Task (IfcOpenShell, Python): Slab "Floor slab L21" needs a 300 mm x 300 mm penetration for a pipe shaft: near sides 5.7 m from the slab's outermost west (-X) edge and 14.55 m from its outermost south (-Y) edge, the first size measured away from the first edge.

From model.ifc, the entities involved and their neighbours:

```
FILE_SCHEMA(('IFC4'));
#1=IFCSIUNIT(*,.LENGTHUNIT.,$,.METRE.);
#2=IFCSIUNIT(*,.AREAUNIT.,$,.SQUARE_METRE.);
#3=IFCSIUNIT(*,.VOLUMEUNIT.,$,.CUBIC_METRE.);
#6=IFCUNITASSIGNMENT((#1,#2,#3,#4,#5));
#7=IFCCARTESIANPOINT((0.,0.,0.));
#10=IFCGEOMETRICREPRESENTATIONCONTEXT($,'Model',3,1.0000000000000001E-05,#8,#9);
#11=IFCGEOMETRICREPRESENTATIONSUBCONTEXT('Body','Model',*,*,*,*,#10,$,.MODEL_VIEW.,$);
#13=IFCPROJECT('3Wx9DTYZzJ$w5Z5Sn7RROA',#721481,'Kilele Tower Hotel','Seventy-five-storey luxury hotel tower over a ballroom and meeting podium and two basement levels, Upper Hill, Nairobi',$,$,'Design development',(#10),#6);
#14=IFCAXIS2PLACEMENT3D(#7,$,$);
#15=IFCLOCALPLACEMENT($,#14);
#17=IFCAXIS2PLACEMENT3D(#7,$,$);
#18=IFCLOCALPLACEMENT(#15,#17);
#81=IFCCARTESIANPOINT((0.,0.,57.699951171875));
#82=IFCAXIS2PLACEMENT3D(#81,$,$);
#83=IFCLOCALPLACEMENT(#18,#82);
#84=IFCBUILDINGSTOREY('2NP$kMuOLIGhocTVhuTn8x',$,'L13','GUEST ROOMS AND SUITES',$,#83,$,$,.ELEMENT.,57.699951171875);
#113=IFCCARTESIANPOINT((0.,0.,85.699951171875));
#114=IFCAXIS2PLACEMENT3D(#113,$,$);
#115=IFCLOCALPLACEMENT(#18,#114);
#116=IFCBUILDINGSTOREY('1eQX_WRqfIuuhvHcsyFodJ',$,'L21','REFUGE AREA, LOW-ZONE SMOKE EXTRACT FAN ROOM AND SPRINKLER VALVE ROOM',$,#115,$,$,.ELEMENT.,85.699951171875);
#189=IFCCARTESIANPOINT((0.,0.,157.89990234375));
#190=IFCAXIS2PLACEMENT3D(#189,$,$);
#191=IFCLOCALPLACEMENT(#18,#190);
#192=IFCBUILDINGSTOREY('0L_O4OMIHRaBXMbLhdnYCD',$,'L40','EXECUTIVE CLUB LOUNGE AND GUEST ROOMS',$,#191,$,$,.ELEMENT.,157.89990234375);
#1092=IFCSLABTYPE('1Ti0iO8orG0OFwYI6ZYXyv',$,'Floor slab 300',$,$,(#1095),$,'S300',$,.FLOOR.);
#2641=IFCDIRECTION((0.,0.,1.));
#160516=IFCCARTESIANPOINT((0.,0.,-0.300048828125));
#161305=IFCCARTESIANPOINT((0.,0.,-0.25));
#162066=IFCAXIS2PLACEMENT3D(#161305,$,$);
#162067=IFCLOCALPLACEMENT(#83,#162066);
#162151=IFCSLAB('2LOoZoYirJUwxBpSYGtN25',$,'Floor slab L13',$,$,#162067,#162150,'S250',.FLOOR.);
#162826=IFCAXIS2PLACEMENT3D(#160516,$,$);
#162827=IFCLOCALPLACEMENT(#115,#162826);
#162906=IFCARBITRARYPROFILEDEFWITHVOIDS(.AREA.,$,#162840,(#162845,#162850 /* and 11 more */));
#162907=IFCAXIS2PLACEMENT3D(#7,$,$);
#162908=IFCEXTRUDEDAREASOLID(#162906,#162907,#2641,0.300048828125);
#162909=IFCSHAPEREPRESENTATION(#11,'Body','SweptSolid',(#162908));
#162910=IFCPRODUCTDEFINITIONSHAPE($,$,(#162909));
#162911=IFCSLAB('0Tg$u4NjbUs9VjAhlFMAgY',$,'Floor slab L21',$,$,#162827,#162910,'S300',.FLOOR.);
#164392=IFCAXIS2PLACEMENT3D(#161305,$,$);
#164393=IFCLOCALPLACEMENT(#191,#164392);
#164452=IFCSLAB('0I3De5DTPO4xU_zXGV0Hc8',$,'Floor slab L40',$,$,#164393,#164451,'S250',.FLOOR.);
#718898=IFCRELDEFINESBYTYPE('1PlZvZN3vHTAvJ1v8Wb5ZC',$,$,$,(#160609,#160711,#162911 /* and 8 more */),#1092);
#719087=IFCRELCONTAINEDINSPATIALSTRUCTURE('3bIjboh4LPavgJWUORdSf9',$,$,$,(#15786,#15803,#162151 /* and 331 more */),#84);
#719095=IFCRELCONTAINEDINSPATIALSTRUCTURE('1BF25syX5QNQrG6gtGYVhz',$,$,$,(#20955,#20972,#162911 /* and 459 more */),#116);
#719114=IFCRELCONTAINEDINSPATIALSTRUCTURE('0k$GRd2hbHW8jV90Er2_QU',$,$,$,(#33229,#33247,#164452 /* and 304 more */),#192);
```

```python
import numpy as np
import ifcopenshell
import ifcopenshell.api.feature
import ifcopenshell.api.geometry
import ifcopenshell.api.root
import ifcopenshell.geom
import ifcopenshell.util.placement
import ifcopenshell.util.representation
import ifcopenshell.util.shape
import ifcopenshell.util.unit

model = ifcopenshell.open("model.ifc")
unit_scale = ifcopenshell.util.unit.calculate_unit_scale(model)
settings = ifcopenshell.geom.settings()


def volume(element):
    """Net volume in cubic metres, openings subtracted."""
    shape = ifcopenshell.geom.create_shape(settings, element)
    return ifcopenshell.util.shape.get_volume(shape.geometry)


slab = model.by_guid("0Tg$u4NjbUs9VjAhlFMAgY")
before = volume(slab)

# Extent in the slab's own axes, in metres. The edges named are its -X and -Y sides.
slab_shape = ifcopenshell.geom.create_shape(settings, slab)
vertices = ifcopenshell.util.shape.get_vertices(slab_shape.geometry)
x_min, y_min, bottom = vertices.min(axis=0)
top = vertices[:, 2].max()

opening = ifcopenshell.api.root.create_entity(model, ifc_class="IfcOpeningElement", name="Pipe shaft opening", predefined_type="OPENING")
context = ifcopenshell.util.representation.get_context(model, "Model", "Body", "MODEL_VIEW")
width, depth = 0.3, 0.3
outline = [(0.0, 0.0), (width, 0.0), (width, depth), (0.0, depth), (0.0, 0.0)]
# Overshoot both faces by 50 mm so the cut is clean.
shape = ifcopenshell.api.geometry.add_slab_representation(
    model, context=context, depth=top - bottom + 0.1, polyline=outline
)
ifcopenshell.api.geometry.assign_representation(model, product=opening, representation=shape)

matrix = ifcopenshell.util.placement.get_local_placement(slab.ObjectPlacement)
matrix[:, 3] = matrix @ np.append(np.array([x_min + 5.7, y_min + 14.55, bottom - 0.05]) / unit_scale, 1.0)
ifcopenshell.api.geometry.edit_object_placement(model, product=opening, matrix=matrix, is_si=False)
ifcopenshell.api.feature.add_feature(model, feature=opening, element=slab)

after = volume(slab)

print(f"slab volume {before:.3f} -> {after:.3f} m3")

model.write("model-out.ifc")
```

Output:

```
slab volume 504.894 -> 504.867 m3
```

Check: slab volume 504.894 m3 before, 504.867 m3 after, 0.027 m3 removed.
